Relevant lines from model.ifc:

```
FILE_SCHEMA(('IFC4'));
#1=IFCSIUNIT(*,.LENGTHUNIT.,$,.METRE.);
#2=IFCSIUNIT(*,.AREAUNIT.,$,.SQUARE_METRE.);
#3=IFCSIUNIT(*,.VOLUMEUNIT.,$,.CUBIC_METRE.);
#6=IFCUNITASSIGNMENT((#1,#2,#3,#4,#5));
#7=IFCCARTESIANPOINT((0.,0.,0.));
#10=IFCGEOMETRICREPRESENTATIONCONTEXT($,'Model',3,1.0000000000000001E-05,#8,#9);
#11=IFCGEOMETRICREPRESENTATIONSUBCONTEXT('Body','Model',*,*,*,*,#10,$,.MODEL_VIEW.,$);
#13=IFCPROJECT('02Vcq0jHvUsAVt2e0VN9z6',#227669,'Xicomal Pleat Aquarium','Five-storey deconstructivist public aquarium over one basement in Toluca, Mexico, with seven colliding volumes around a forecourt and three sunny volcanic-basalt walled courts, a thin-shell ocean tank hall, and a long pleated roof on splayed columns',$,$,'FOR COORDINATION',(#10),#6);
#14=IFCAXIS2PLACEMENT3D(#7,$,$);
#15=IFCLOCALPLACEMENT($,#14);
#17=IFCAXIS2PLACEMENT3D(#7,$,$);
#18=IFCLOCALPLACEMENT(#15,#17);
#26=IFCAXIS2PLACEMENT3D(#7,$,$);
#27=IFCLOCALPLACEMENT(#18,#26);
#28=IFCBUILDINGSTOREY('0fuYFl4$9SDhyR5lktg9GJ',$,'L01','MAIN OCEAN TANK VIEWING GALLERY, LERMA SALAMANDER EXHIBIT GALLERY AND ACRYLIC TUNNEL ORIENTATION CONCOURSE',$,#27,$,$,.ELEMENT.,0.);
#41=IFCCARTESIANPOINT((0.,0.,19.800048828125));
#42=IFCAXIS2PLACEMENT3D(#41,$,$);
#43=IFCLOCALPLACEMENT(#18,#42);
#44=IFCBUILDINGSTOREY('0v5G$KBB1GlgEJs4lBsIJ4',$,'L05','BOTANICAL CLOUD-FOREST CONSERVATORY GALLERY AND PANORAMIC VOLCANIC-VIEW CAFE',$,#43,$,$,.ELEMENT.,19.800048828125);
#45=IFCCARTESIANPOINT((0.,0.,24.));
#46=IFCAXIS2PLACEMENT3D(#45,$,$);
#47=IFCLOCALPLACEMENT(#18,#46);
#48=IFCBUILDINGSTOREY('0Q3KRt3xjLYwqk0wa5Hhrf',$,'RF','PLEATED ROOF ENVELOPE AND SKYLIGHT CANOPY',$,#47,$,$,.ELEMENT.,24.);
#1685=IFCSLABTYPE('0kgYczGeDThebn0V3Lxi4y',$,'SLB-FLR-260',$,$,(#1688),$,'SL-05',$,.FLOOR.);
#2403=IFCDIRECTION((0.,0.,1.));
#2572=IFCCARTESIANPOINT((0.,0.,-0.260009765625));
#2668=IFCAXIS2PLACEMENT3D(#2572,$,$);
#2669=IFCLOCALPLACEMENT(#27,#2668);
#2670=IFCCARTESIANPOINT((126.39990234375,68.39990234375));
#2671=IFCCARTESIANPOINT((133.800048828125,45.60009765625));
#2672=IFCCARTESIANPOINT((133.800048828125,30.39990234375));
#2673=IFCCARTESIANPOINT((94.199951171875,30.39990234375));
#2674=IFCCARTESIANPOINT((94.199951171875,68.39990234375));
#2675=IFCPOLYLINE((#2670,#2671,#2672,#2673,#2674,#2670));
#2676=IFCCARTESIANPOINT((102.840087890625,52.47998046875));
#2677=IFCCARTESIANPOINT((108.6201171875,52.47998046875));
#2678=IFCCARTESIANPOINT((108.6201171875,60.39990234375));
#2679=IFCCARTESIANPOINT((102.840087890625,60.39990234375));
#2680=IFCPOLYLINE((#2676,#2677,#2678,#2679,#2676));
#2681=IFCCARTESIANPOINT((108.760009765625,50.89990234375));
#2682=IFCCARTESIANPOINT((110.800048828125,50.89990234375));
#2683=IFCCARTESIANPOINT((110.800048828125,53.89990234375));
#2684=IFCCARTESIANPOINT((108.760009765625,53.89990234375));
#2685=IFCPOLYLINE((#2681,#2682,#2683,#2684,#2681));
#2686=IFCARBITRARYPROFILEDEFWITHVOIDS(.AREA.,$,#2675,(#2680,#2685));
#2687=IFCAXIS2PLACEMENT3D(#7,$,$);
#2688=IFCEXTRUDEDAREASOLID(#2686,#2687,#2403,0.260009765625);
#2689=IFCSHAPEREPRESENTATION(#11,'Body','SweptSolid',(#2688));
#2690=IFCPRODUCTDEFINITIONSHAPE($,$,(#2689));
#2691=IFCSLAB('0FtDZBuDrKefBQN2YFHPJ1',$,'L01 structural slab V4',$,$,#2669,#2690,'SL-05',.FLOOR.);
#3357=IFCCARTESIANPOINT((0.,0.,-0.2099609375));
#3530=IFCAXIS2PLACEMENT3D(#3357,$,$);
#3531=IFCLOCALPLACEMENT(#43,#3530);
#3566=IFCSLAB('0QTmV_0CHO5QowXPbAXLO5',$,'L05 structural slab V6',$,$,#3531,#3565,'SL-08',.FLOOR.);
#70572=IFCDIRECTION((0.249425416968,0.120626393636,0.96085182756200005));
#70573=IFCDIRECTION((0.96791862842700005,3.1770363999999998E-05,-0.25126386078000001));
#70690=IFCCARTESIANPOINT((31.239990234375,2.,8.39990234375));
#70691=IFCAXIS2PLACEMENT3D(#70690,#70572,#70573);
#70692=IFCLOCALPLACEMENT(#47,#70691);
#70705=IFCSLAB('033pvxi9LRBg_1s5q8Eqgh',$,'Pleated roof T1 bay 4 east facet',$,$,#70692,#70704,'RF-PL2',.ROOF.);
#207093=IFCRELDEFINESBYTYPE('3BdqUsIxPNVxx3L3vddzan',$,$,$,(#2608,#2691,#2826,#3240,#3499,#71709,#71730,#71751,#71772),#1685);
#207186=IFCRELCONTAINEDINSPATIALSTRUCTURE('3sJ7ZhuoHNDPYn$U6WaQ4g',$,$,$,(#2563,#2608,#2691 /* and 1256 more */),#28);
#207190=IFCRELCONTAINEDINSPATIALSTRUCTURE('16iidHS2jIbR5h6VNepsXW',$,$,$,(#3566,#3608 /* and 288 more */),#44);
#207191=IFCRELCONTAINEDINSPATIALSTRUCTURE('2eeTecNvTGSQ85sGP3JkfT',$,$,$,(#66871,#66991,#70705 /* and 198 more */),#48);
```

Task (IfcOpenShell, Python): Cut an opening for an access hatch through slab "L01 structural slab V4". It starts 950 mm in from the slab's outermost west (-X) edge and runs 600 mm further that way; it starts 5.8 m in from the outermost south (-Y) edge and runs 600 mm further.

```python
import numpy as np
import ifcopenshell
import ifcopenshell.api.feature
import ifcopenshell.api.geometry
import ifcopenshell.api.root
import ifcopenshell.geom
import ifcopenshell.util.placement
import ifcopenshell.util.representation
import ifcopenshell.util.shape
import ifcopenshell.util.unit

model = ifcopenshell.open("model.ifc")
unit_scale = ifcopenshell.util.unit.calculate_unit_scale(model)
settings = ifcopenshell.geom.settings()


def volume(element):
    """Net volume in cubic metres, openings subtracted."""
    shape = ifcopenshell.geom.create_shape(settings, element)
    return ifcopenshell.util.shape.get_volume(shape.geometry)


slab = model.by_id(2691)
before = volume(slab)

# Extent in the slab's own axes, in metres. The edges named are its -X and -Y sides.
slab_shape = ifcopenshell.geom.create_shape(settings, slab)
vertices = ifcopenshell.util.shape.get_vertices(slab_shape.geometry)
x_min, y_min, bottom = vertices.min(axis=0)
top = vertices[:, 2].max()

opening = ifcopenshell.api.root.create_entity(model, ifc_class="IfcOpeningElement", name="Access hatch opening", predefined_type="OPENING")
context = ifcopenshell.util.representation.get_context(model, "Model", "Body", "MODEL_VIEW")
width, depth = 0.6, 0.6
outline = [(0.0, 0.0), (width, 0.0), (width, depth), (0.0, depth), (0.0, 0.0)]
# Overshoot both faces by 50 mm so the cut is clean.
shape = ifcopenshell.api.geometry.add_slab_representation(
    model, context=context, depth=top - bottom + 0.1, polyline=outline
)
ifcopenshell.api.geometry.assign_representation(model, product=opening, representation=shape)

matrix = ifcopenshell.util.placement.get_local_placement(slab.ObjectPlacement)
matrix[:, 3] = matrix @ np.append(np.array([x_min + 0.95, y_min + 5.8, bottom - 0.05]) / unit_scale, 1.0)
ifcopenshell.api.geometry.edit_object_placement(model, product=opening, matrix=matrix, is_si=False)
ifcopenshell.api.feature.add_feature(model, feature=opening, element=slab)

after = volume(slab)

print(f"slab volume {before:.3f} -> {after:.3f} m3")

model.write("model-out.ifc")
```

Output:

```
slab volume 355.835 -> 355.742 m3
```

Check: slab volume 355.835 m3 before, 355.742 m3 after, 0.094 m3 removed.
